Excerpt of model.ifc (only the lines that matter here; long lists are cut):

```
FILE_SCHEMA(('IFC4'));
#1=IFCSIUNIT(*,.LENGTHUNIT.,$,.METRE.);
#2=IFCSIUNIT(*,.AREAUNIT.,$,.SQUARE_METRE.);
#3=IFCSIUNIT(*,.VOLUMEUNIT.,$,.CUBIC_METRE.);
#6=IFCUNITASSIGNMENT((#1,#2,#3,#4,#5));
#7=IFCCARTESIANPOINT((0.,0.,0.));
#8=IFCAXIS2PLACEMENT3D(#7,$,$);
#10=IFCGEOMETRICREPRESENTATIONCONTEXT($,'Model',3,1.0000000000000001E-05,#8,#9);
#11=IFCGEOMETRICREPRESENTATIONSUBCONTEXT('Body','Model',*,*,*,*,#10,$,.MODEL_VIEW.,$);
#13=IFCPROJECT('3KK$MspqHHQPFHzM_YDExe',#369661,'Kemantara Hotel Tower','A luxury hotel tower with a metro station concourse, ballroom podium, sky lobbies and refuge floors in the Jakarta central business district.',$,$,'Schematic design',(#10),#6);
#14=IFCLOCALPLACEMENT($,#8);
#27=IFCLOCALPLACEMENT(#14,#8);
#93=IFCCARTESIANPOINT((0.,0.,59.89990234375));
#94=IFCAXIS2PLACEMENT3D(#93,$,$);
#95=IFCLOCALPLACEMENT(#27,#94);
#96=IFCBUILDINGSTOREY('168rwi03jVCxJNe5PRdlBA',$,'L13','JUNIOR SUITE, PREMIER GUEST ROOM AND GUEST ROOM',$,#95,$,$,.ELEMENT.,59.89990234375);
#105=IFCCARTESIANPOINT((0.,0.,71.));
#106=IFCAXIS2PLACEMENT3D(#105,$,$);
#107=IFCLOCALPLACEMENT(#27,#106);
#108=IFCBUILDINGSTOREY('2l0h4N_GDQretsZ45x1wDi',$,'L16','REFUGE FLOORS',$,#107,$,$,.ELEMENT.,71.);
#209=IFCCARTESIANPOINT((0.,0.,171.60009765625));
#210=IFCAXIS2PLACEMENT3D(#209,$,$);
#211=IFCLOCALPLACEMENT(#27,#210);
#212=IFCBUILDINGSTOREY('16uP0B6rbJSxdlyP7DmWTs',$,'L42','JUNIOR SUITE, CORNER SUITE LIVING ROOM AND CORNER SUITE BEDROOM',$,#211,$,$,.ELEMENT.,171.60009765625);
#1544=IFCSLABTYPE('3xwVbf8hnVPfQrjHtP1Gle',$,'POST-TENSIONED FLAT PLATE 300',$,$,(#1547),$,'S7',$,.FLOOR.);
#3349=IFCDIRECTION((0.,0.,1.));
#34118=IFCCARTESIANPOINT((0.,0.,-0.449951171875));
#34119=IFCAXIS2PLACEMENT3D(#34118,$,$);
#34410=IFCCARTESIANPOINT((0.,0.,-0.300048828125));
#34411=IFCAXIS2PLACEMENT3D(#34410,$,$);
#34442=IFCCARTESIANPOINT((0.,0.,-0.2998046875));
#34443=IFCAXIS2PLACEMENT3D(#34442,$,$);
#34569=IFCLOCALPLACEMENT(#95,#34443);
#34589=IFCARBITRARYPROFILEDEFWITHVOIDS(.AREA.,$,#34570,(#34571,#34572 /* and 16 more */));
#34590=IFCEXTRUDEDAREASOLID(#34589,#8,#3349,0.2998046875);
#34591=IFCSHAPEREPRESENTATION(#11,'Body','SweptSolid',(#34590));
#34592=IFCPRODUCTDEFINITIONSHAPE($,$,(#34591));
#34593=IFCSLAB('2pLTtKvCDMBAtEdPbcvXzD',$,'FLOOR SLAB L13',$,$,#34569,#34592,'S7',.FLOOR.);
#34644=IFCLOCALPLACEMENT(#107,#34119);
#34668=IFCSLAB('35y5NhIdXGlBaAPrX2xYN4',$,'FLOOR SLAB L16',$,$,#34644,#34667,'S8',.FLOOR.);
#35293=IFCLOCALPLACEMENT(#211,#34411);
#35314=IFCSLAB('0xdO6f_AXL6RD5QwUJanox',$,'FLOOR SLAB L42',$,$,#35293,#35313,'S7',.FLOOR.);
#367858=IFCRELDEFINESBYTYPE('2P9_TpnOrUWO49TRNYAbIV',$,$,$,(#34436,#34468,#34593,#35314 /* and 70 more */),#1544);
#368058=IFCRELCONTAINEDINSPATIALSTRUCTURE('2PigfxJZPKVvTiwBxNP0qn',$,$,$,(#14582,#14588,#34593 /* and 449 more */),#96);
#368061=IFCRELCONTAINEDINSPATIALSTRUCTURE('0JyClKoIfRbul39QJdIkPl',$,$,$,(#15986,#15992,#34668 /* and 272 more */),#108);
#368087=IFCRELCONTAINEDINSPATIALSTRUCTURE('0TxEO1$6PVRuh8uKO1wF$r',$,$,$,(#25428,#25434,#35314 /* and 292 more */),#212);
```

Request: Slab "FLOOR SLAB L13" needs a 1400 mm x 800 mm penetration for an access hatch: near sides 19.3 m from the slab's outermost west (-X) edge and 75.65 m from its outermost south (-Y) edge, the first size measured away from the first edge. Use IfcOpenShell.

```python
import numpy as np
import ifcopenshell
import ifcopenshell.api.feature
import ifcopenshell.api.geometry
import ifcopenshell.api.root
import ifcopenshell.geom
import ifcopenshell.util.placement
import ifcopenshell.util.representation
import ifcopenshell.util.shape
import ifcopenshell.util.unit

model = ifcopenshell.open("model.ifc")
unit_scale = ifcopenshell.util.unit.calculate_unit_scale(model)
settings = ifcopenshell.geom.settings()


def volume(element):
    """Net volume in cubic metres, openings subtracted."""
    shape = ifcopenshell.geom.create_shape(settings, element)
    return ifcopenshell.util.shape.get_volume(shape.geometry)


slab = model.by_guid("2pLTtKvCDMBAtEdPbcvXzD")
before = volume(slab)

# Extent in the slab's own axes, in metres. The edges named are its -X and -Y sides.
slab_shape = ifcopenshell.geom.create_shape(settings, slab)
vertices = ifcopenshell.util.shape.get_vertices(slab_shape.geometry)
x_min, y_min, bottom = vertices.min(axis=0)
top = vertices[:, 2].max()

opening = ifcopenshell.api.root.create_entity(model, ifc_class="IfcOpeningElement", name="Access hatch opening", predefined_type="OPENING")
context = ifcopenshell.util.representation.get_context(model, "Model", "Body", "MODEL_VIEW")
width, depth = 1.4, 0.8
outline = [(0.0, 0.0), (width, 0.0), (width, depth), (0.0, depth), (0.0, 0.0)]
# Overshoot both faces by 50 mm so the cut is clean.
shape = ifcopenshell.api.geometry.add_slab_representation(
    model, context=context, depth=top - bottom + 0.1, polyline=outline
)
ifcopenshell.api.geometry.assign_representation(model, product=opening, representation=shape)

matrix = ifcopenshell.util.placement.get_local_placement(slab.ObjectPlacement)
matrix[:, 3] = matrix @ np.append(np.array([x_min + 19.3, y_min + 75.65, bottom - 0.05]) / unit_scale, 1.0)
ifcopenshell.api.geometry.edit_object_placement(model, product=opening, matrix=matrix, is_si=False)
ifcopenshell.api.feature.add_feature(model, feature=opening, element=slab)

after = volume(slab)

print(f"slab volume {before:.3f} -> {after:.3f} m3")

model.write("model-out.ifc")
```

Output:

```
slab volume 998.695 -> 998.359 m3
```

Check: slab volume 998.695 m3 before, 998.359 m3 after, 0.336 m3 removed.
